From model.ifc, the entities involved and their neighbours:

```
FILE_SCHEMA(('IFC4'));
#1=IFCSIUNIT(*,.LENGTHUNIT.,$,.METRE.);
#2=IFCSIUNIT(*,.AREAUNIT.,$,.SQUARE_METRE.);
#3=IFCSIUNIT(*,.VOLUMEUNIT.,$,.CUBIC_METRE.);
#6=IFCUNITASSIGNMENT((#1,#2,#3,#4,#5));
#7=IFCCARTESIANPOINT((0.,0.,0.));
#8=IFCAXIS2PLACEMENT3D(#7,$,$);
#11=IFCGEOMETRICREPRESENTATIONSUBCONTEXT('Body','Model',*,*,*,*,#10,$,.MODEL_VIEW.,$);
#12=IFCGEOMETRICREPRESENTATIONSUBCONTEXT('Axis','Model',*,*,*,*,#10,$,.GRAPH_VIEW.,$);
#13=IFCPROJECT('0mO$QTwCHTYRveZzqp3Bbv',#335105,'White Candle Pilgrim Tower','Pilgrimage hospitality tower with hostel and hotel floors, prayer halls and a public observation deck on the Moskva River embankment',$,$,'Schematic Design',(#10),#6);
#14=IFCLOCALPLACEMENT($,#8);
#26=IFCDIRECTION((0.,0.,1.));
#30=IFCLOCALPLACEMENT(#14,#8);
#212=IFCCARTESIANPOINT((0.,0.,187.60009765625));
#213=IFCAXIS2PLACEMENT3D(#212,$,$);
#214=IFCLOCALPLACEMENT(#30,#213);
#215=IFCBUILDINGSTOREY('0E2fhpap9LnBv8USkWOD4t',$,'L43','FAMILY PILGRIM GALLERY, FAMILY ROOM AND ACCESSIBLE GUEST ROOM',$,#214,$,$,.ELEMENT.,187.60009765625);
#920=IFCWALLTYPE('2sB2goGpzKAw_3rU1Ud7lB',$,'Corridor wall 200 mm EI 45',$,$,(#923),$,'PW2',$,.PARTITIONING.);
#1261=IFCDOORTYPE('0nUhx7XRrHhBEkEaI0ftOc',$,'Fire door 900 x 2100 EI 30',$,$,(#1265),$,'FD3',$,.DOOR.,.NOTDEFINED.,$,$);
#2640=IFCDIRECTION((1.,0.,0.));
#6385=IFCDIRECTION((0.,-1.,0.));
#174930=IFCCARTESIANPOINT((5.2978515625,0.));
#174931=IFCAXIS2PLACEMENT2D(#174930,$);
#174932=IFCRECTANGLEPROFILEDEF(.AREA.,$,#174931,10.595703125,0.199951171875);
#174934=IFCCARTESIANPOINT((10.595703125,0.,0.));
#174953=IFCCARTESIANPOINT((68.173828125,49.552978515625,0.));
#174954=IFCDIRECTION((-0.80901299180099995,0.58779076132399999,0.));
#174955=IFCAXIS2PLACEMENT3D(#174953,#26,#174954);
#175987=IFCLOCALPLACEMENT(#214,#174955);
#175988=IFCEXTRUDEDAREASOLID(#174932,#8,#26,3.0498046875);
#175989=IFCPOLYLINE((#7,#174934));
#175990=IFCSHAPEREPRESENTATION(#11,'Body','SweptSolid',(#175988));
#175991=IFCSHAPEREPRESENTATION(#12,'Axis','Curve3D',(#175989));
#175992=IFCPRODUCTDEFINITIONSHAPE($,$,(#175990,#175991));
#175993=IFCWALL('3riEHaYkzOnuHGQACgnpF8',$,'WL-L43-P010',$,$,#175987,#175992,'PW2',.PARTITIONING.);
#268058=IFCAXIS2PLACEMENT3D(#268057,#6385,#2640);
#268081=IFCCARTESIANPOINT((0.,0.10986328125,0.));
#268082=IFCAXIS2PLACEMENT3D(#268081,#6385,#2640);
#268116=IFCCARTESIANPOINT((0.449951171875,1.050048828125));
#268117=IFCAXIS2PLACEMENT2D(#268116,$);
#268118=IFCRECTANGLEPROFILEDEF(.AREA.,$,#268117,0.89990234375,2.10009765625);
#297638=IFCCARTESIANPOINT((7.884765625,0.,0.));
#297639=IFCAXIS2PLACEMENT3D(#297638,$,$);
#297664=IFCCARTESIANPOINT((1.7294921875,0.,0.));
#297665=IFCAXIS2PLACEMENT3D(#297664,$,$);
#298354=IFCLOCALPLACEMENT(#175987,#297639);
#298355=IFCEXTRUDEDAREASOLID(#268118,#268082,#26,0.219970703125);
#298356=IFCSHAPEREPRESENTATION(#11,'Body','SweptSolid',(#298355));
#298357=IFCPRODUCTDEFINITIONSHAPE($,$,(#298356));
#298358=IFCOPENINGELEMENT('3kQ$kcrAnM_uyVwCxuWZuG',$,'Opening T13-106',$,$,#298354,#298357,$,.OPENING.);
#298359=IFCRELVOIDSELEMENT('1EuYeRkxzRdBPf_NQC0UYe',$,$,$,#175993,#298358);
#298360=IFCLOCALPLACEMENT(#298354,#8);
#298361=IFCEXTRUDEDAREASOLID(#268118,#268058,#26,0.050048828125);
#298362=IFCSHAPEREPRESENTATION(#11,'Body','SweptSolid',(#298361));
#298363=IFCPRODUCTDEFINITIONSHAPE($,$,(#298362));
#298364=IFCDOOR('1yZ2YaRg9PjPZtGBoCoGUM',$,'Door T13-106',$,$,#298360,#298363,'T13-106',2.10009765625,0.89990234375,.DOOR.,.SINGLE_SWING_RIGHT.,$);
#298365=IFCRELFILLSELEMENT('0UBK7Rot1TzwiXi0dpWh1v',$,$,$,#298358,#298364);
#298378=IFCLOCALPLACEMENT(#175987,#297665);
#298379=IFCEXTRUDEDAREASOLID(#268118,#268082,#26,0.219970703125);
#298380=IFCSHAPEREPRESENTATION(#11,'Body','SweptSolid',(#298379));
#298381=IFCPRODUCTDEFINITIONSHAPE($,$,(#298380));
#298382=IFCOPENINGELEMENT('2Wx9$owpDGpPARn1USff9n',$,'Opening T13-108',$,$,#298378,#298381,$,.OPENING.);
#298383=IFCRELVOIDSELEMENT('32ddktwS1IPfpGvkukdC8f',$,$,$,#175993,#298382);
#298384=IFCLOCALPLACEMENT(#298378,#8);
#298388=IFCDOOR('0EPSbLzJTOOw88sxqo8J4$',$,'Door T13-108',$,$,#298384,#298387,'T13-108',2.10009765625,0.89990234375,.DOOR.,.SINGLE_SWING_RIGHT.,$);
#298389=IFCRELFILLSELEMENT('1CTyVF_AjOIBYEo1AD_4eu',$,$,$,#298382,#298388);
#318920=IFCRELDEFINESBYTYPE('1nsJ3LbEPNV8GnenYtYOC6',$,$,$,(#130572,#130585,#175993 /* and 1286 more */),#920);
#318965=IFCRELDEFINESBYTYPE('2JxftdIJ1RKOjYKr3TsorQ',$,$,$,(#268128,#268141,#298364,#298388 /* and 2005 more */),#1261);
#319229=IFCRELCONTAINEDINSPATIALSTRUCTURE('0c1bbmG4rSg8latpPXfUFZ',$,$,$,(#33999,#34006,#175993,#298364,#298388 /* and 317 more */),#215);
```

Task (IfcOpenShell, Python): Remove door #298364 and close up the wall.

```python
import ifcopenshell
import ifcopenshell.api.feature
import ifcopenshell.api.root
import ifcopenshell.geom
import ifcopenshell.util.shape

model = ifcopenshell.open("model.ifc")
settings = ifcopenshell.geom.settings()


def volume(element):
    """Net volume in cubic metres, openings subtracted."""
    shape = ifcopenshell.geom.create_shape(settings, element)
    return ifcopenshell.util.shape.get_volume(shape.geometry)


door = model.by_id(298364)
opening = door.FillsVoids[0].RelatingOpeningElement
wall = opening.VoidsElements[0].RelatingBuildingElement
before = volume(wall)

ifcopenshell.api.root.remove_product(model, product=door)
ifcopenshell.api.feature.remove_feature(model, feature=opening)

after = volume(wall)

print(f"wall volume {before:.3f} -> {after:.3f} m3")

model.write("model-out.ifc")
```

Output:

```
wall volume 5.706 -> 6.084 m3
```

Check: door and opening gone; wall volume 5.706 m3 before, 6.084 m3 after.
